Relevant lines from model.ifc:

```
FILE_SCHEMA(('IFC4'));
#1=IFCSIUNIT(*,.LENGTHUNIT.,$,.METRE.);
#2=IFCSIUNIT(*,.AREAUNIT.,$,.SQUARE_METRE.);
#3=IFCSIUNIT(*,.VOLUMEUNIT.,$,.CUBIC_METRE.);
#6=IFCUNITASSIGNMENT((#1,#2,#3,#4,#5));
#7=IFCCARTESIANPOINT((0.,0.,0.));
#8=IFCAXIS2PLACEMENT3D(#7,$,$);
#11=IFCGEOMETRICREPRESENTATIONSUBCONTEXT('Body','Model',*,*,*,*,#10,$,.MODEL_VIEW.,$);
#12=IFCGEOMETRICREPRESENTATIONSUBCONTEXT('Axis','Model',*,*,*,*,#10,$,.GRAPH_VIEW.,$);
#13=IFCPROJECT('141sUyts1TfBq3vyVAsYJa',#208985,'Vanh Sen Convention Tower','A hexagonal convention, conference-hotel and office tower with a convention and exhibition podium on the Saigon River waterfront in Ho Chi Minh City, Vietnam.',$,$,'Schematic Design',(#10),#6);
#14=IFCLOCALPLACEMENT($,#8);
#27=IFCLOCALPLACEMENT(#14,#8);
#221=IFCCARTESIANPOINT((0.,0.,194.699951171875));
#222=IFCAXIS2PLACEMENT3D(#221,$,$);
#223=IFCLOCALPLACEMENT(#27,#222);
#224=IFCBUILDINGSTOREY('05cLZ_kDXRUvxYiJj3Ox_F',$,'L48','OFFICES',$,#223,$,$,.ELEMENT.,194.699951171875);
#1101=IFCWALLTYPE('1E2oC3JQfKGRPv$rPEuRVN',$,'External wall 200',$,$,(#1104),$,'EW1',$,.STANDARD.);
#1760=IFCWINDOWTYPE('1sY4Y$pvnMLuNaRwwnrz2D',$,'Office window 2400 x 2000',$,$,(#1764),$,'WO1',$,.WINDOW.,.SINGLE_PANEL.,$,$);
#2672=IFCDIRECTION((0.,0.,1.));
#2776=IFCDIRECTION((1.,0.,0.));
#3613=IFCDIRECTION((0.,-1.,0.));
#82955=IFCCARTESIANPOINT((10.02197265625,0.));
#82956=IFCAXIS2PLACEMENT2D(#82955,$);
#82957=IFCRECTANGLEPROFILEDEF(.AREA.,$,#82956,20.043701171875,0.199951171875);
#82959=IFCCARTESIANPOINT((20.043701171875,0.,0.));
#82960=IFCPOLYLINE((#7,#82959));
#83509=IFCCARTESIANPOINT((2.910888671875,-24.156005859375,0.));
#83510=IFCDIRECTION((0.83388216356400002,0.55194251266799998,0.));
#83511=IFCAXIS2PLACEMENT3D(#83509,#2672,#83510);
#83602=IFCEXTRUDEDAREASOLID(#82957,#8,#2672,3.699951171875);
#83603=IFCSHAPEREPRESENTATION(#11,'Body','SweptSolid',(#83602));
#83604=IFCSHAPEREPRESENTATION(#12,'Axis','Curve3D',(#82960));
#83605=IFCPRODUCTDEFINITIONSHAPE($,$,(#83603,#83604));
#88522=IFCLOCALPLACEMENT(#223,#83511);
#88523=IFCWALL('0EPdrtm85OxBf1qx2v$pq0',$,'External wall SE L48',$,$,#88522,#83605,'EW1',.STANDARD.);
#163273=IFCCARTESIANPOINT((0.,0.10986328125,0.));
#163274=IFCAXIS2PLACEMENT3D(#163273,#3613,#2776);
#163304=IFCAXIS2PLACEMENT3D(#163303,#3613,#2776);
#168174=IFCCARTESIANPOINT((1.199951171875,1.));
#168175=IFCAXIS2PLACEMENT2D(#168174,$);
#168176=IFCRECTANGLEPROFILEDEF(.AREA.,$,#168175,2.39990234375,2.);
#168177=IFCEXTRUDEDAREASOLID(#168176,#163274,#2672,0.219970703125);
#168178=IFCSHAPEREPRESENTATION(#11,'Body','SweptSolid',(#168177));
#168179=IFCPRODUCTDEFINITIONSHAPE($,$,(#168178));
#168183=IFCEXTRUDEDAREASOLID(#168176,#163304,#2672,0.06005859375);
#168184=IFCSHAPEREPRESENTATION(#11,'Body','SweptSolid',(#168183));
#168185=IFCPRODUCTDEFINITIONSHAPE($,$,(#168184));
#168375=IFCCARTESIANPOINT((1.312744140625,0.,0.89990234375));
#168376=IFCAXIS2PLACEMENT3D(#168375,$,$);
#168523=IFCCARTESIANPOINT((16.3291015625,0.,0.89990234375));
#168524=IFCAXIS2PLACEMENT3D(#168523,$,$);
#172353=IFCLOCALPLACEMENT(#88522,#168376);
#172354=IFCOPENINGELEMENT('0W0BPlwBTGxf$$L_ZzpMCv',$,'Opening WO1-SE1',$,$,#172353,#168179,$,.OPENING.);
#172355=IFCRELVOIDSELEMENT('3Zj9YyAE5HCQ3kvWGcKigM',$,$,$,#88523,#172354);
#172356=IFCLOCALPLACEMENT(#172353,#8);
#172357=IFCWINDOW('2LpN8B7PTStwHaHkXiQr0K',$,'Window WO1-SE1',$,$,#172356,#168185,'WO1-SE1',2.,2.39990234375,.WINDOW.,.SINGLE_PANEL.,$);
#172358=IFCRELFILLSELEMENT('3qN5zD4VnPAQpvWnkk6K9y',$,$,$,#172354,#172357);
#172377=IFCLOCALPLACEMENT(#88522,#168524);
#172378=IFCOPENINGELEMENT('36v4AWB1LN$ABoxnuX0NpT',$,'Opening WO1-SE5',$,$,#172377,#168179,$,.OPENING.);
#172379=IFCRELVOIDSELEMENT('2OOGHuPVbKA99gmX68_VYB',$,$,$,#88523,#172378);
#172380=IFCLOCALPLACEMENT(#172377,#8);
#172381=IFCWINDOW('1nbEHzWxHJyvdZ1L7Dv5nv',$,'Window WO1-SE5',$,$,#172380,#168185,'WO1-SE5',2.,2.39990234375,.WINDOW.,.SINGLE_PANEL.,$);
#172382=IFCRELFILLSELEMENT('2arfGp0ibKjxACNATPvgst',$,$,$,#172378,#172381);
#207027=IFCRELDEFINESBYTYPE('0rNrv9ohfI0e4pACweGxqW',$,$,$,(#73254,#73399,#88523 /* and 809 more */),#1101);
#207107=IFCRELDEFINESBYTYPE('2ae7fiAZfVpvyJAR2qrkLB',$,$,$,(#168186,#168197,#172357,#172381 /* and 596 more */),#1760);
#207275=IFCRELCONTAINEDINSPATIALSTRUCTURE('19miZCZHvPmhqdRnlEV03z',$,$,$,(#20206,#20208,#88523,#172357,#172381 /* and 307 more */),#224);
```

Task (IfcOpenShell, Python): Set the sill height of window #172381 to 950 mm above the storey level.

```python
import numpy as np
import ifcopenshell
import ifcopenshell.api.geometry
import ifcopenshell.geom
import ifcopenshell.util.element
import ifcopenshell.util.placement
import ifcopenshell.util.shape
import ifcopenshell.util.unit

model = ifcopenshell.open("model.ifc")
unit_scale = ifcopenshell.util.unit.calculate_unit_scale(model)

window = model.by_guid("1nbEHzWxHJyvdZ1L7Dv5nv")
opening = window.FillsVoids[0].RelatingOpeningElement
storey = ifcopenshell.util.element.get_container(window, ifc_class="IfcBuildingStorey")
level = ifcopenshell.util.placement.get_local_placement(storey.ObjectPlacement)[2, 3]

# The opening's origin need not be at the sill, so measure its lowest point.
shape = ifcopenshell.geom.create_shape(ifcopenshell.geom.settings(), opening)
bottom = ifcopenshell.util.shape.get_shape_bottom_elevation(shape, shape.geometry) / unit_scale
dz = level + 0.95 - bottom

shift = np.array([0.0, 0.0, dz])
# The window is placed relative to its opening, so it follows when the opening moves.
matrix = ifcopenshell.util.placement.get_local_placement(opening.ObjectPlacement)
matrix[:3, 3] += shift
ifcopenshell.api.geometry.edit_object_placement(
    model, product=opening, matrix=matrix, is_si=False, should_transform_children=True
)

print(f"moved by {dz * unit_scale:+.3f} m")

model.write("model_updated.ifc")
```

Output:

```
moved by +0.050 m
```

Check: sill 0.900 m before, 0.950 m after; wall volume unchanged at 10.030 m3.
